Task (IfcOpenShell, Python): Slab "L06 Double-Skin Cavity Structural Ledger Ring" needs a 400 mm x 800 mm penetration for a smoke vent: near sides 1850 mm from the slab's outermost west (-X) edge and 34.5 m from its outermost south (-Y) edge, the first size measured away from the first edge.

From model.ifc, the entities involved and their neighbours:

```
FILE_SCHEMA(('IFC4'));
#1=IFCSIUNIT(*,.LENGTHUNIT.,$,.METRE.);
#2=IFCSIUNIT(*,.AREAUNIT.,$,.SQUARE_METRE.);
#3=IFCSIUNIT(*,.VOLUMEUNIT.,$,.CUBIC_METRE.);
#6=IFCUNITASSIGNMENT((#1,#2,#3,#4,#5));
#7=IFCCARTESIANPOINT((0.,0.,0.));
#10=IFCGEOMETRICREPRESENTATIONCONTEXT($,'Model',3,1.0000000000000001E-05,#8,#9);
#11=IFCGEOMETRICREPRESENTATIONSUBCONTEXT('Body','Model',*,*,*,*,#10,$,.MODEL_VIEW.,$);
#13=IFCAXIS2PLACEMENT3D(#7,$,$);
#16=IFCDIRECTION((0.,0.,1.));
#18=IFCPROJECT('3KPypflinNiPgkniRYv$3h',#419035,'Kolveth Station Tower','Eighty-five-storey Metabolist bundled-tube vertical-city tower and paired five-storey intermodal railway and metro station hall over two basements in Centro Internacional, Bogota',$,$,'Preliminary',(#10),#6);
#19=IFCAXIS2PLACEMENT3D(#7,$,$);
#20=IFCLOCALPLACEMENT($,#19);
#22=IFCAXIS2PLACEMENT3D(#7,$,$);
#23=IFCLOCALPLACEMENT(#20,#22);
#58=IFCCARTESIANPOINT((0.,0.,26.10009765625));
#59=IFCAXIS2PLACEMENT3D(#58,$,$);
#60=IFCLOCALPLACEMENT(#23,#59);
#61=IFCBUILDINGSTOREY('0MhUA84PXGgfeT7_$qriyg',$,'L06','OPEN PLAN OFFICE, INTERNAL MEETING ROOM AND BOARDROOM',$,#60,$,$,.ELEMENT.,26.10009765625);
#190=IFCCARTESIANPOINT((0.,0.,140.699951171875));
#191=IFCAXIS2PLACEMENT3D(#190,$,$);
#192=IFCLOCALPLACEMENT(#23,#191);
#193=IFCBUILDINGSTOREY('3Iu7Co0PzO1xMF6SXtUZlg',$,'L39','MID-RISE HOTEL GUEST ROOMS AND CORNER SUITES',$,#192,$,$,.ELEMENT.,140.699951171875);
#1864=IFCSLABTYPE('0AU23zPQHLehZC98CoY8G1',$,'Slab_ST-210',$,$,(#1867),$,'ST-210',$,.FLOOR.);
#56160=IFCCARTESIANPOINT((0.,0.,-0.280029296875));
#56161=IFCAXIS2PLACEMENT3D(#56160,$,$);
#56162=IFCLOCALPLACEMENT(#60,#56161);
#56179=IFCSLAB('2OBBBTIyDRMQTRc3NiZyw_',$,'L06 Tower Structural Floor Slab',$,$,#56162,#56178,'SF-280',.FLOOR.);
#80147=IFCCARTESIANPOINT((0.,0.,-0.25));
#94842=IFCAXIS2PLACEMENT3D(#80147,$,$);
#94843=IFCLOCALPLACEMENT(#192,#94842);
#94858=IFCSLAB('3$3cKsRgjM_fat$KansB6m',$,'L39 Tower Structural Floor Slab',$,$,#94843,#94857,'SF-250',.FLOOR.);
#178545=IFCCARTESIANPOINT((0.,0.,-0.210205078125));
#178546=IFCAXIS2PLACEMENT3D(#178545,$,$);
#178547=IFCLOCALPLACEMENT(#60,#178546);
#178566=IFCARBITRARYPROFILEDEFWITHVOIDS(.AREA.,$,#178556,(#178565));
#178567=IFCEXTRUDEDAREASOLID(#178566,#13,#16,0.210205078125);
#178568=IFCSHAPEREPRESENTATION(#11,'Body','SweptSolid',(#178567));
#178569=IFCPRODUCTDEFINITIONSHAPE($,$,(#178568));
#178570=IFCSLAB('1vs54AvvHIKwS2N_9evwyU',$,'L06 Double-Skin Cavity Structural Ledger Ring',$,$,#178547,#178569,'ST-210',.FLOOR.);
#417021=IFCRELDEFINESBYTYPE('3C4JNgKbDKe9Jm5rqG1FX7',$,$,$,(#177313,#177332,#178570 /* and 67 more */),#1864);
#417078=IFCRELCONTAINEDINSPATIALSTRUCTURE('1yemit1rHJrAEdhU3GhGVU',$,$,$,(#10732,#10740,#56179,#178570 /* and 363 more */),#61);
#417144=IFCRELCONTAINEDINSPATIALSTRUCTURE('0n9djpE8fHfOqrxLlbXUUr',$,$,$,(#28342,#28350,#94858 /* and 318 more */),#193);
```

```python
import numpy as np
import ifcopenshell
import ifcopenshell.api.feature
import ifcopenshell.api.geometry
import ifcopenshell.api.root
import ifcopenshell.geom
import ifcopenshell.util.placement
import ifcopenshell.util.representation
import ifcopenshell.util.shape
import ifcopenshell.util.unit

model = ifcopenshell.open("model.ifc")
unit_scale = ifcopenshell.util.unit.calculate_unit_scale(model)
settings = ifcopenshell.geom.settings()


def volume(element):
    """Net volume in cubic metres, openings subtracted."""
    shape = ifcopenshell.geom.create_shape(settings, element)
    return ifcopenshell.util.shape.get_volume(shape.geometry)


slab = model.by_guid("1vs54AvvHIKwS2N_9evwyU")
before = volume(slab)

# Extent in the slab's own axes, in metres. The edges named are its -X and -Y sides.
slab_shape = ifcopenshell.geom.create_shape(settings, slab)
vertices = ifcopenshell.util.shape.get_vertices(slab_shape.geometry)
x_min, y_min, bottom = vertices.min(axis=0)
top = vertices[:, 2].max()

opening = ifcopenshell.api.root.create_entity(model, ifc_class="IfcOpeningElement", name="Smoke vent opening", predefined_type="OPENING")
context = ifcopenshell.util.representation.get_context(model, "Model", "Body", "MODEL_VIEW")
width, depth = 0.4, 0.8
outline = [(0.0, 0.0), (width, 0.0), (width, depth), (0.0, depth), (0.0, 0.0)]
# Overshoot both faces by 50 mm so the cut is clean.
shape = ifcopenshell.api.geometry.add_slab_representation(
    model, context=context, depth=top - bottom + 0.1, polyline=outline
)
ifcopenshell.api.geometry.assign_representation(model, product=opening, representation=shape)

matrix = ifcopenshell.util.placement.get_local_placement(slab.ObjectPlacement)
matrix[:, 3] = matrix @ np.append(np.array([x_min + 1.85, y_min + 34.5, bottom - 0.05]) / unit_scale, 1.0)
ifcopenshell.api.geometry.edit_object_placement(model, product=opening, matrix=matrix, is_si=False)
ifcopenshell.api.feature.add_feature(model, feature=opening, element=slab)

after = volume(slab)

print(f"slab volume {before:.3f} -> {after:.3f} m3")

model.write("model_edited.ifc")
```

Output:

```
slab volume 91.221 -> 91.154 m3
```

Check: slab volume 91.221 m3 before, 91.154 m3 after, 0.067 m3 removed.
